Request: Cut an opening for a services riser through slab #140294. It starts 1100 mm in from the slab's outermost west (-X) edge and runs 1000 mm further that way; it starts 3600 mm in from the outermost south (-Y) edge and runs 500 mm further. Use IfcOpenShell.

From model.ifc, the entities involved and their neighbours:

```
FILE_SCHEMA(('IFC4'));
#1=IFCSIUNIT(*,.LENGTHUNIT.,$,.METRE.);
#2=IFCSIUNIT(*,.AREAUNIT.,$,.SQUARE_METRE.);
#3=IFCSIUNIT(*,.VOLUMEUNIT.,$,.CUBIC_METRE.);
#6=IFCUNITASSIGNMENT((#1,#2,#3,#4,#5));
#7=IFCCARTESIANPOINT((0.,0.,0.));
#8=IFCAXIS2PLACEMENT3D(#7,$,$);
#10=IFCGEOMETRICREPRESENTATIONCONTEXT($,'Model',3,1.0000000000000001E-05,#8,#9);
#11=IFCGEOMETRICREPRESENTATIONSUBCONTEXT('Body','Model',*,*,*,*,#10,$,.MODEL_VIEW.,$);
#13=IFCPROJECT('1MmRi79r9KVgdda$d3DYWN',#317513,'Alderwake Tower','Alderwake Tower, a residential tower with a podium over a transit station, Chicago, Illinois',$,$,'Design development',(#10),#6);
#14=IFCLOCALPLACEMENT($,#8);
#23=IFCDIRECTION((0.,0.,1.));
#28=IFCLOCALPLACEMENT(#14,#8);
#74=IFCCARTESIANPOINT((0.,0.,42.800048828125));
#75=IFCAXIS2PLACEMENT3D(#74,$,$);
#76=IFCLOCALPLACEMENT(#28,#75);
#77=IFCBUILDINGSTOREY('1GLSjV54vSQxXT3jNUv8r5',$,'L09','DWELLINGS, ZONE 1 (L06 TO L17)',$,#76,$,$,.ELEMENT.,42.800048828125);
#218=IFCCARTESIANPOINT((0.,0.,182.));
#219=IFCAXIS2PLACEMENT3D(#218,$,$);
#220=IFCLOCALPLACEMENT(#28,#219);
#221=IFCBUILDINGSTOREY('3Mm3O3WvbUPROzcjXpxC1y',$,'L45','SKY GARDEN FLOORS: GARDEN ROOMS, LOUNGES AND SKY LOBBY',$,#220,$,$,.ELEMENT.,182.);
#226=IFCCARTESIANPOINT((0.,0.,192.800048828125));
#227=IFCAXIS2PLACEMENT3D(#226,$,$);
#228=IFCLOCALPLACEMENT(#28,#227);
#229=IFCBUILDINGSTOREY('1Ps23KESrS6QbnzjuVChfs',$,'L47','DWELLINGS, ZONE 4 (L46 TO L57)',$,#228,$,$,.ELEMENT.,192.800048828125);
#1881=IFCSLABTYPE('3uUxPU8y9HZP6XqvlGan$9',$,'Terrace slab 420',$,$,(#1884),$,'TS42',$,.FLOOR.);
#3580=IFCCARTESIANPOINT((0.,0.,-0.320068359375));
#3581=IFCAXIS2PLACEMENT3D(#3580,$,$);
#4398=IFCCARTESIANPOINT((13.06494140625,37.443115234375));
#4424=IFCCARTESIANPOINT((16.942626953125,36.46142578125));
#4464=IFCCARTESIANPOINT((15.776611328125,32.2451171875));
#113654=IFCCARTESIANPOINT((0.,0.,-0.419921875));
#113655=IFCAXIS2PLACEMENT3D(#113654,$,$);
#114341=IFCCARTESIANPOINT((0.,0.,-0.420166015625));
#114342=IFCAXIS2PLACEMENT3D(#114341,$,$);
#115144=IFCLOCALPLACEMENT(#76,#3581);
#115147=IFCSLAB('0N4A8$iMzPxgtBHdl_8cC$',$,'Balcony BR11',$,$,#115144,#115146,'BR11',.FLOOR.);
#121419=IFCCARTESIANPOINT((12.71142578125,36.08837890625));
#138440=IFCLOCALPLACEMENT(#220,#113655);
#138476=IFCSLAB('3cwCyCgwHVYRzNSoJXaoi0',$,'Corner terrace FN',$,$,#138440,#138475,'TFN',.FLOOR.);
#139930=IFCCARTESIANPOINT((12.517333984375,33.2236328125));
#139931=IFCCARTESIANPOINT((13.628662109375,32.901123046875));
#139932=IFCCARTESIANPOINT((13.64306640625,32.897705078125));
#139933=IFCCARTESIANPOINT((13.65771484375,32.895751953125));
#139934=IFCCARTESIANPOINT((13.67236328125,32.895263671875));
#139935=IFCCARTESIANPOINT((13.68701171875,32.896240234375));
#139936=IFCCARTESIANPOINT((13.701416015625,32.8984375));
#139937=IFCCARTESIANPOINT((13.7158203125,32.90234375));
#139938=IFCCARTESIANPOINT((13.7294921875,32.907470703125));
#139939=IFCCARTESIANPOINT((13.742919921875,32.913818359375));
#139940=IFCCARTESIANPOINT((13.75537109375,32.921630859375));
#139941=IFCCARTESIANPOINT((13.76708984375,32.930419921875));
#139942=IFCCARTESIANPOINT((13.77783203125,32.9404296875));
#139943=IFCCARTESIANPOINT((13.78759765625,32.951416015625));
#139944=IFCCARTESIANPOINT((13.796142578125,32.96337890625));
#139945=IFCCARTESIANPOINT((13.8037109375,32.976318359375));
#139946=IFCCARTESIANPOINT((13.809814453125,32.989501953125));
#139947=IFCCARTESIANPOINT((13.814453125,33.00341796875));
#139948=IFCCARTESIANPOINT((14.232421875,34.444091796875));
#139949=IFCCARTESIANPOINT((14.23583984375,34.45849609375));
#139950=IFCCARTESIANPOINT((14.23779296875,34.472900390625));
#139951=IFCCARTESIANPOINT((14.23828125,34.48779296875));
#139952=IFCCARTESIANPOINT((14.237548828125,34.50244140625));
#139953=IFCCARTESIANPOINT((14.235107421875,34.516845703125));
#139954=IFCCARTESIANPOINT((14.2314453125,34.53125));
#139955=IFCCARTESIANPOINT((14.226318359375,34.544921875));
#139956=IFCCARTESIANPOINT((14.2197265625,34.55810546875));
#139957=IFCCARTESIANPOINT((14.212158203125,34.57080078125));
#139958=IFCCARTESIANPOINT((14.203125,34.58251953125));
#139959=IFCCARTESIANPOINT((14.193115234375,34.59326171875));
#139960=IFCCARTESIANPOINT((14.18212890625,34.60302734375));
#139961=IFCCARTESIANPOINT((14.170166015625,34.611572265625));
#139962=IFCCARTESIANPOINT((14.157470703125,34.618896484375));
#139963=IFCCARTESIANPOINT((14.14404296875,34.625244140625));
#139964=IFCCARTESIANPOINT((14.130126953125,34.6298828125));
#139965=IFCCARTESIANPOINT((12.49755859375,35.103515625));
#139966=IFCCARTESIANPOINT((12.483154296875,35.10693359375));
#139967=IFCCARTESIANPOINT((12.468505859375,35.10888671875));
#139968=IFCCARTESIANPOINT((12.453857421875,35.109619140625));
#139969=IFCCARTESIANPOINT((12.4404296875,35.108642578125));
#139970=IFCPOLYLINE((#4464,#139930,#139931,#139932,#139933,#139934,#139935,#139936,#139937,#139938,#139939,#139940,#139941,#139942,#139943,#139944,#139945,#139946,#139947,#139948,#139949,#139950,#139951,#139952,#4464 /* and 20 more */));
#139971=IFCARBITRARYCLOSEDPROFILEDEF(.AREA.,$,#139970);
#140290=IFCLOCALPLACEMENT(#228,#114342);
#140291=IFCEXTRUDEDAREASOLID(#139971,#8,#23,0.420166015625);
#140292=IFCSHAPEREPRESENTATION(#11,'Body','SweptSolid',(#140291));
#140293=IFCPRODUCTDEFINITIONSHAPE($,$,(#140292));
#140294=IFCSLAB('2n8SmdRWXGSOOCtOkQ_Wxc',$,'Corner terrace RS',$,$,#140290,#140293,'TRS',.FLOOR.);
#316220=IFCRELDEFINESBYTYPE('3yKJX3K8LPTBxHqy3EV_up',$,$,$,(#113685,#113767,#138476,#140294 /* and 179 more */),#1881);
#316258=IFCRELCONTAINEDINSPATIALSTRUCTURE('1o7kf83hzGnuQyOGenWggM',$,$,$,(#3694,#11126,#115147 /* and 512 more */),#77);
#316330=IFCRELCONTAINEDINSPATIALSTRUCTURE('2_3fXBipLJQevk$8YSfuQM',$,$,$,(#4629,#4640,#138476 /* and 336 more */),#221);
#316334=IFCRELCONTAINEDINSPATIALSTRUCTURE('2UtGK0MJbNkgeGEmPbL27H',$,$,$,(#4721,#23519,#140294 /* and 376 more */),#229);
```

```python
import numpy as np
import ifcopenshell
import ifcopenshell.api.feature
import ifcopenshell.api.geometry
import ifcopenshell.api.root
import ifcopenshell.geom
import ifcopenshell.util.placement
import ifcopenshell.util.representation
import ifcopenshell.util.shape
import ifcopenshell.util.unit

model = ifcopenshell.open("model.ifc")
unit_scale = ifcopenshell.util.unit.calculate_unit_scale(model)
settings = ifcopenshell.geom.settings()


def volume(element):
    """Net volume in cubic metres, openings subtracted."""
    shape = ifcopenshell.geom.create_shape(settings, element)
    return ifcopenshell.util.shape.get_volume(shape.geometry)


slab = model.by_id(140294)
before = volume(slab)

# Extent in the slab's own axes, in metres. The edges named are its -X and -Y sides.
slab_shape = ifcopenshell.geom.create_shape(settings, slab)
vertices = ifcopenshell.util.shape.get_vertices(slab_shape.geometry)
x_min, y_min, bottom = vertices.min(axis=0)
top = vertices[:, 2].max()

opening = ifcopenshell.api.root.create_entity(model, ifc_class="IfcOpeningElement", name="Services riser opening", predefined_type="OPENING")
context = ifcopenshell.util.representation.get_context(model, "Model", "Body", "MODEL_VIEW")
width, depth = 1, 0.5
outline = [(0.0, 0.0), (width, 0.0), (width, depth), (0.0, depth), (0.0, 0.0)]
# Overshoot both faces by 50 mm so the cut is clean.
shape = ifcopenshell.api.geometry.add_slab_representation(
    model, context=context, depth=top - bottom + 0.1, polyline=outline
)
ifcopenshell.api.geometry.assign_representation(model, product=opening, representation=shape)

matrix = ifcopenshell.util.placement.get_local_placement(slab.ObjectPlacement)
matrix[:, 3] = matrix @ np.append(np.array([x_min + 1.1, y_min + 3.6, bottom - 0.05]) / unit_scale, 1.0)
ifcopenshell.api.geometry.edit_object_placement(model, product=opening, matrix=matrix, is_si=False)
ifcopenshell.api.feature.add_feature(model, feature=opening, element=slab)

after = volume(slab)

print(f"slab volume {before:.3f} -> {after:.3f} m3")

model.write("model_v2.ifc")
```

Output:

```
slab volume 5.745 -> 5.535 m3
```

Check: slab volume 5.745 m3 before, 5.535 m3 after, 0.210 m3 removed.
